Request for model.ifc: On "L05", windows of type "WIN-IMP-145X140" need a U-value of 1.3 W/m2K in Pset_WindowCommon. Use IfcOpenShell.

First a look at what the model holds.

```python
import ifcopenshell
import ifcopenshell.util.element

model = ifcopenshell.open("model.ifc")
print(model.schema)
storey = next(s for s in model.by_type("IfcBuildingStorey") if s.Name == "L05")
windows = [e for e in ifcopenshell.util.element.get_decomposition(storey) if e.is_a("IfcWindow")]
seen = {}
for e in windows:
    element_type = ifcopenshell.util.element.get_type(e)
    key = (element_type.Name if element_type != e and element_type else None, ifcopenshell.util.element.get_pset(e, "Pset_WindowCommon", "ThermalTransmittance"))
    seen[key] = seen.get(key, 0) + 1
for (name, value), count in sorted(seen.items(), key=str):
    print(count, "x", name, "|", value)
```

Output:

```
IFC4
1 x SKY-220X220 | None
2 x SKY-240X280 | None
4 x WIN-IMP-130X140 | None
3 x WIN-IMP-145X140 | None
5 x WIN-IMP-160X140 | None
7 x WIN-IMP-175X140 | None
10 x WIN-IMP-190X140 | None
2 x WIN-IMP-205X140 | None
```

```python
import ifcopenshell
import ifcopenshell.api.pset
import ifcopenshell.util.element

model = ifcopenshell.open("model.ifc")

storey = next(s for s in model.by_type("IfcBuildingStorey") if s.Name == "L05")
windows = [e for e in ifcopenshell.util.element.get_decomposition(storey) if e.is_a("IfcWindow")]

count = 0
for e in windows:
    element_type = ifcopenshell.util.element.get_type(e)
    if element_type in (None, e) or element_type.Name != "WIN-IMP-145X140":
        continue
    # add_pset returns the element's existing set when there is one.
    pset = ifcopenshell.api.pset.add_pset(model, product=e, name="Pset_WindowCommon")
    ifcopenshell.api.pset.edit_pset(model, pset=pset, properties={"ThermalTransmittance": 1.3})
    count += 1

print(count, "windows updated")

model.write("model_updated.ifc")
```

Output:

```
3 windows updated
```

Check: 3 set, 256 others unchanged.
